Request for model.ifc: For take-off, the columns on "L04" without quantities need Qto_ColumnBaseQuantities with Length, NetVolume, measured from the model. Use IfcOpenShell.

First a look at what the model holds.

```python
import ifcopenshell
import ifcopenshell.util.element
import ifcopenshell.util.unit

model = ifcopenshell.open("model.ifc")
print(model.schema)
for unit_type in ("LENGTHUNIT", "AREAUNIT", "VOLUMEUNIT"):
    print(unit_type, ifcopenshell.util.unit.calculate_unit_scale(model, unit_type))
storey = next(s for s in model.by_type("IfcBuildingStorey") if s.Name == "L04")
columns = [e for e in ifcopenshell.util.element.get_decomposition(storey) if e.is_a("IfcColumn")]
for e in sorted(columns, key=lambda e: e.id()):
    print(e.id(), e.is_a(), e.Name, list(ifcopenshell.util.element.get_psets(e, qtos_only=True)), sep=" | ")
```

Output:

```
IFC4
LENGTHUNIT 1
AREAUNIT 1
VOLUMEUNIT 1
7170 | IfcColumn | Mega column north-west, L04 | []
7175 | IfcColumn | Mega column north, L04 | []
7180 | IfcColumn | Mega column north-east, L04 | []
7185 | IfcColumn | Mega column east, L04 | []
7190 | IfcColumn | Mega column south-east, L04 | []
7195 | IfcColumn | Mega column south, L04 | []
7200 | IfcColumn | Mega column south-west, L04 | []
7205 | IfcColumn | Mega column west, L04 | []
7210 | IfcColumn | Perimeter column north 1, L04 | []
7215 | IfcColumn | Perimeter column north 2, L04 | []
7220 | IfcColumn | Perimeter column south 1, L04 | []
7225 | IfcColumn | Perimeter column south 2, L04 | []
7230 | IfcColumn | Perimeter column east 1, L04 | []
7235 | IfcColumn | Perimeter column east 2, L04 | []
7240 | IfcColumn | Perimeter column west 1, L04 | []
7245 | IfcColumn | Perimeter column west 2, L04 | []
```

```python
import ifcopenshell
import ifcopenshell.api.pset
import ifcopenshell.geom
import ifcopenshell.util.element
import ifcopenshell.util.shape
import ifcopenshell.util.unit

model = ifcopenshell.open("model.ifc")
unit_scale = ifcopenshell.util.unit.calculate_unit_scale(model)
volume_scale = ifcopenshell.util.unit.calculate_unit_scale(model, "VOLUMEUNIT")
settings = ifcopenshell.geom.settings()

storey = next(s for s in model.by_type("IfcBuildingStorey") if s.Name == "L04")
columns = [e for e in ifcopenshell.util.element.get_decomposition(storey) if e.is_a("IfcColumn")]

for e in sorted(columns, key=lambda e: e.id()):
    if ifcopenshell.util.element.get_psets(e, qtos_only=True, should_inherit=False):
        continue
    # Geometry comes back in metres, in the element's own axes.
    shape = ifcopenshell.geom.create_shape(settings, e)
    values = {
        "Length": ifcopenshell.util.shape.get_z(shape.geometry) / unit_scale,
        "NetVolume": ifcopenshell.util.shape.get_volume(shape.geometry) / volume_scale,
    }
    qto = ifcopenshell.api.pset.add_qto(model, product=e, name="Qto_ColumnBaseQuantities")
    ifcopenshell.api.pset.edit_qto(model, qto=qto, properties=values)
    print(e.id(), {k: round(v, 3) for k, v in values.items()})

model.write("model_rev.ifc")
```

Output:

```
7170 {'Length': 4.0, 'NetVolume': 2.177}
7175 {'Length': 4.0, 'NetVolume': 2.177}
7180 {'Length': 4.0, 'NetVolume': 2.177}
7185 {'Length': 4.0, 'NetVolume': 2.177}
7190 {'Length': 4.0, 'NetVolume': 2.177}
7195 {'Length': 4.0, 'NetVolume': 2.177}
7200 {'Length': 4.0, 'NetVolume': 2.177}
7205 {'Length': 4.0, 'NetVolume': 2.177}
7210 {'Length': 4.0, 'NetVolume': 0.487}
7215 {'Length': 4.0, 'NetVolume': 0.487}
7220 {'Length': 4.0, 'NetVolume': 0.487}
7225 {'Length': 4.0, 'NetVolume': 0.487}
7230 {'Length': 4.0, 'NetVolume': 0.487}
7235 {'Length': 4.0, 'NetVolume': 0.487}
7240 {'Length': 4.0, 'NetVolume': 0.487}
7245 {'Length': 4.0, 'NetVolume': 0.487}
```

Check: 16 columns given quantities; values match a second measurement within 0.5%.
